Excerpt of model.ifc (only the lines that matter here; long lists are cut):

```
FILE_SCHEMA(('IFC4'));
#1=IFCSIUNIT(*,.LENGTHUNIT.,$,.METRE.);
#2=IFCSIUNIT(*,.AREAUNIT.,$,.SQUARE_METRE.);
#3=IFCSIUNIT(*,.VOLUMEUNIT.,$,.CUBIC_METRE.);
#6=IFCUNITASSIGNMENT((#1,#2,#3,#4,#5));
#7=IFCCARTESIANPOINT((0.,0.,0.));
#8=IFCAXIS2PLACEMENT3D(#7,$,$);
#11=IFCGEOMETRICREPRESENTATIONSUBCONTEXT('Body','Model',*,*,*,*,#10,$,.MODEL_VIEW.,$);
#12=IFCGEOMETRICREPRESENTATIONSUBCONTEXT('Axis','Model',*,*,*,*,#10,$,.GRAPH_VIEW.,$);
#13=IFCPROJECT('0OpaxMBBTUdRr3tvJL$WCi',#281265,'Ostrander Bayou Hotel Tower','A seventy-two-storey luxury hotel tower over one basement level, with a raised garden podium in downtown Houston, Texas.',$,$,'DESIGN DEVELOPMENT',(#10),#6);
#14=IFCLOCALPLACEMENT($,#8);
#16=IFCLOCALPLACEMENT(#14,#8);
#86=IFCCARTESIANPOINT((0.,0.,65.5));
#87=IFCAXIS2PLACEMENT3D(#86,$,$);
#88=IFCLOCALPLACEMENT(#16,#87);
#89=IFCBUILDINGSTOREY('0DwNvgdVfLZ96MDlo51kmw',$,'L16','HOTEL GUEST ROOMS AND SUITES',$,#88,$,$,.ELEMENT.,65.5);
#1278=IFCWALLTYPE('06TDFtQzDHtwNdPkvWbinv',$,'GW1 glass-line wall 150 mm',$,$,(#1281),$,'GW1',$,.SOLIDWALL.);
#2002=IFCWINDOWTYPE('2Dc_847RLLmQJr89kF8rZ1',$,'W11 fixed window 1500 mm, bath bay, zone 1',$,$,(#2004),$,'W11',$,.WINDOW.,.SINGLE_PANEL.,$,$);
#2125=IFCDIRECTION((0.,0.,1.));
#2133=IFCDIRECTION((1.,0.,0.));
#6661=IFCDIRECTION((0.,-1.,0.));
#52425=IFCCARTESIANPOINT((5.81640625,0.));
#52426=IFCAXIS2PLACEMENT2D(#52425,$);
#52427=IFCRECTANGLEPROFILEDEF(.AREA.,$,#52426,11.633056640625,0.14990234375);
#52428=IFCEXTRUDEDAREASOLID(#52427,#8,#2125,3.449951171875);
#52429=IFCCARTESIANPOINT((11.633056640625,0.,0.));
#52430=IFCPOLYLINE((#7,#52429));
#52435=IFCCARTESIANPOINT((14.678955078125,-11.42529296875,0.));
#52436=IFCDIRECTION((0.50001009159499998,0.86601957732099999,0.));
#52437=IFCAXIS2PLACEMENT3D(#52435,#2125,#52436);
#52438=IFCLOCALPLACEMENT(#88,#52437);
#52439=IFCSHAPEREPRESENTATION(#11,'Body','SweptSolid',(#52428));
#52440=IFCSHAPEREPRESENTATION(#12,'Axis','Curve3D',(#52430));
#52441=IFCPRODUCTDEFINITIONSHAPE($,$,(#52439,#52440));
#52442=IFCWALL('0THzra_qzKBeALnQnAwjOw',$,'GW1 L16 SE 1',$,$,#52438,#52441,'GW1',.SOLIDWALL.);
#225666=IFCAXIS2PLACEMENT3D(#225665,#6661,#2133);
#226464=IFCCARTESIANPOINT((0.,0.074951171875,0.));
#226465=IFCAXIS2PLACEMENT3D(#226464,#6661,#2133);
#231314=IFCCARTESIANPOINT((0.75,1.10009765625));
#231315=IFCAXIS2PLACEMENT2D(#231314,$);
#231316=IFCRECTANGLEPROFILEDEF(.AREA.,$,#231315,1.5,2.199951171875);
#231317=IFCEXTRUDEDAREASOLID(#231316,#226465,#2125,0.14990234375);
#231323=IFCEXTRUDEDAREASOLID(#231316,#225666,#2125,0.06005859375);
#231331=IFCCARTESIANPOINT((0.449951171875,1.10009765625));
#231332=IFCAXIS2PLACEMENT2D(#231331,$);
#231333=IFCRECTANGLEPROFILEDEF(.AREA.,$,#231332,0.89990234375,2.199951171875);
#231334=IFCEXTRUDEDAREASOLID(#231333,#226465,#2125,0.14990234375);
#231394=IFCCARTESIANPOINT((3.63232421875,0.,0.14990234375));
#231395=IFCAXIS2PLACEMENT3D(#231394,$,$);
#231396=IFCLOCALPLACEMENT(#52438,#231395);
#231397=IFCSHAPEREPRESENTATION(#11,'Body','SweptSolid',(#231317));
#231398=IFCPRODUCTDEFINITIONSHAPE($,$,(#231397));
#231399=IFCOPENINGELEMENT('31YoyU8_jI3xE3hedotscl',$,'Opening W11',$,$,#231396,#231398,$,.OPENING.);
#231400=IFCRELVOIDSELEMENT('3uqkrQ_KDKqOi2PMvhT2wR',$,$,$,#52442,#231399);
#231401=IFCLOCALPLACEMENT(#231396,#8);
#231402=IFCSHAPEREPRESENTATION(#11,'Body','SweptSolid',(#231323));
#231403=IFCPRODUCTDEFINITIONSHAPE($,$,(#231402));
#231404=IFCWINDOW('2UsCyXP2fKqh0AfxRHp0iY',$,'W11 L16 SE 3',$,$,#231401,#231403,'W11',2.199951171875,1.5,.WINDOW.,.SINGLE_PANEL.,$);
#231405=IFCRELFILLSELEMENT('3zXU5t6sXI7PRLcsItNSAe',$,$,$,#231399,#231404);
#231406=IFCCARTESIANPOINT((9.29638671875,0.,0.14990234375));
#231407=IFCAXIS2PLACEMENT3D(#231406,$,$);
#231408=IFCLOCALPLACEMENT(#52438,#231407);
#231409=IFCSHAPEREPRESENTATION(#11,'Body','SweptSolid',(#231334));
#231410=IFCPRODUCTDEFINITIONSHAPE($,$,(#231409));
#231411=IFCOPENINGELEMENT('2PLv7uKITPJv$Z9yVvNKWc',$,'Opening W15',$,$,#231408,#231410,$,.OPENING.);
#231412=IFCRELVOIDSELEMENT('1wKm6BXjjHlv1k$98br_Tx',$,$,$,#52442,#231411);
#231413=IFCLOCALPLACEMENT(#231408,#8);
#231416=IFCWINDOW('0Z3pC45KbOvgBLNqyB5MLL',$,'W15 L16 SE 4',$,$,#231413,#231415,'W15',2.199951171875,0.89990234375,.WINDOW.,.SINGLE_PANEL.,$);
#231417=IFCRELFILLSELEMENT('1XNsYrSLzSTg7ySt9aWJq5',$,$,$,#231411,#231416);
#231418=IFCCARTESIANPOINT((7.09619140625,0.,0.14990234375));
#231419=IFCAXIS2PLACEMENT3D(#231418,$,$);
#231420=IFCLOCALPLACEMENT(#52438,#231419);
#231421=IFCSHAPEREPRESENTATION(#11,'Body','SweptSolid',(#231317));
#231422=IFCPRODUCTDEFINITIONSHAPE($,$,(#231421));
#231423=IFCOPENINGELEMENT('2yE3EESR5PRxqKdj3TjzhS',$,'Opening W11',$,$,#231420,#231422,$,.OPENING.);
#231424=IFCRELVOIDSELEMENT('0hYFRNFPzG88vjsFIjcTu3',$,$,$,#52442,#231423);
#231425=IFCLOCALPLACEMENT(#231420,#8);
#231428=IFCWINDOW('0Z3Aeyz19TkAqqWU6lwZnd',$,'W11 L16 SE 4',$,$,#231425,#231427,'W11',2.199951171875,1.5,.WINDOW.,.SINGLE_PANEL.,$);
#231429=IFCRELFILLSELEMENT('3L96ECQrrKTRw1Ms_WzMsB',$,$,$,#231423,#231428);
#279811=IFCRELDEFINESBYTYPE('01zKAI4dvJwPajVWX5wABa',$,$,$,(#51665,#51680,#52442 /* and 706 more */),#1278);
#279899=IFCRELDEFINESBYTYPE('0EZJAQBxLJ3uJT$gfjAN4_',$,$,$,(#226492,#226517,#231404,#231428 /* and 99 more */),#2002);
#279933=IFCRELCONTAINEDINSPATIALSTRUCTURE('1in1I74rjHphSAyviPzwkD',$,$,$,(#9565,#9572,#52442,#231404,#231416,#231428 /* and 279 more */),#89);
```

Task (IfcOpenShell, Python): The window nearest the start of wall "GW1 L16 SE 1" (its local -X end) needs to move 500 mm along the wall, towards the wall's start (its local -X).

```python
import ifcopenshell
import ifcopenshell.api.geometry
import ifcopenshell.util.placement

model = ifcopenshell.open("model.ifc")

window = model.by_guid("2UsCyXP2fKqh0AfxRHp0iY")
opening = window.FillsVoids[0].RelatingOpeningElement
wall = opening.VoidsElements[0].RelatingBuildingElement

wall_matrix = ifcopenshell.util.placement.get_local_placement(wall.ObjectPlacement)
shift = wall_matrix[:3, 0] * -0.5
before = ifcopenshell.util.placement.get_local_placement(window.ObjectPlacement)[:3, 3].copy()

# The window is placed relative to its opening, so it follows when the opening moves.
matrix = ifcopenshell.util.placement.get_local_placement(opening.ObjectPlacement)
matrix[:3, 3] += shift
ifcopenshell.api.geometry.edit_object_placement(
    model, product=opening, matrix=matrix, is_si=False, should_transform_children=True
)

after = ifcopenshell.util.placement.get_local_placement(window.ObjectPlacement)[:3, 3]
print("window moved by", (after - before).round(3) + 0.0)

model.write("model-out.ifc")
```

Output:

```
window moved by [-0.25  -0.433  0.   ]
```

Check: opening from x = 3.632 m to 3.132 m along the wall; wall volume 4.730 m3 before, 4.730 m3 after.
